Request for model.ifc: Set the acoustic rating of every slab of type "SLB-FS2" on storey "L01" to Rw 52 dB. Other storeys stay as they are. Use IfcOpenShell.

First a look at what the model holds.

```python
import ifcopenshell
import ifcopenshell.util.element

model = ifcopenshell.open("model.ifc")
print(model.schema)
storey = next(s for s in model.by_type("IfcBuildingStorey") if s.Name == "L01")
slabs = [e for e in ifcopenshell.util.element.get_decomposition(storey) if e.is_a("IfcSlab")]
seen = {}
for e in slabs:
    element_type = ifcopenshell.util.element.get_type(e)
    key = (element_type.Name if element_type != e and element_type else None, ifcopenshell.util.element.get_pset(e, "Pset_SlabCommon", "AcousticRating"))
    seen[key] = seen.get(key, 0) + 1
for (name, value), count in sorted(seen.items(), key=str):
    print(count, "x", name, "|", value)
```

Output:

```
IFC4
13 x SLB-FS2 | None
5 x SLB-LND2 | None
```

```python
import ifcopenshell
import ifcopenshell.api.pset
import ifcopenshell.util.element

model = ifcopenshell.open("model.ifc")

storey = next(s for s in model.by_type("IfcBuildingStorey") if s.Name == "L01")
slabs = [e for e in ifcopenshell.util.element.get_decomposition(storey) if e.is_a("IfcSlab")]

count = 0
for e in slabs:
    element_type = ifcopenshell.util.element.get_type(e)
    if element_type in (None, e) or element_type.Name != "SLB-FS2":
        continue
    # add_pset returns the element's existing set when there is one.
    pset = ifcopenshell.api.pset.add_pset(model, product=e, name="Pset_SlabCommon")
    ifcopenshell.api.pset.edit_pset(model, pset=pset, properties={"AcousticRating": "Rw 52 dB"})
    count += 1

print(count, "slabs updated")

model.write("model_edited.ifc")
```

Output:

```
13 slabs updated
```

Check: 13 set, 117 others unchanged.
